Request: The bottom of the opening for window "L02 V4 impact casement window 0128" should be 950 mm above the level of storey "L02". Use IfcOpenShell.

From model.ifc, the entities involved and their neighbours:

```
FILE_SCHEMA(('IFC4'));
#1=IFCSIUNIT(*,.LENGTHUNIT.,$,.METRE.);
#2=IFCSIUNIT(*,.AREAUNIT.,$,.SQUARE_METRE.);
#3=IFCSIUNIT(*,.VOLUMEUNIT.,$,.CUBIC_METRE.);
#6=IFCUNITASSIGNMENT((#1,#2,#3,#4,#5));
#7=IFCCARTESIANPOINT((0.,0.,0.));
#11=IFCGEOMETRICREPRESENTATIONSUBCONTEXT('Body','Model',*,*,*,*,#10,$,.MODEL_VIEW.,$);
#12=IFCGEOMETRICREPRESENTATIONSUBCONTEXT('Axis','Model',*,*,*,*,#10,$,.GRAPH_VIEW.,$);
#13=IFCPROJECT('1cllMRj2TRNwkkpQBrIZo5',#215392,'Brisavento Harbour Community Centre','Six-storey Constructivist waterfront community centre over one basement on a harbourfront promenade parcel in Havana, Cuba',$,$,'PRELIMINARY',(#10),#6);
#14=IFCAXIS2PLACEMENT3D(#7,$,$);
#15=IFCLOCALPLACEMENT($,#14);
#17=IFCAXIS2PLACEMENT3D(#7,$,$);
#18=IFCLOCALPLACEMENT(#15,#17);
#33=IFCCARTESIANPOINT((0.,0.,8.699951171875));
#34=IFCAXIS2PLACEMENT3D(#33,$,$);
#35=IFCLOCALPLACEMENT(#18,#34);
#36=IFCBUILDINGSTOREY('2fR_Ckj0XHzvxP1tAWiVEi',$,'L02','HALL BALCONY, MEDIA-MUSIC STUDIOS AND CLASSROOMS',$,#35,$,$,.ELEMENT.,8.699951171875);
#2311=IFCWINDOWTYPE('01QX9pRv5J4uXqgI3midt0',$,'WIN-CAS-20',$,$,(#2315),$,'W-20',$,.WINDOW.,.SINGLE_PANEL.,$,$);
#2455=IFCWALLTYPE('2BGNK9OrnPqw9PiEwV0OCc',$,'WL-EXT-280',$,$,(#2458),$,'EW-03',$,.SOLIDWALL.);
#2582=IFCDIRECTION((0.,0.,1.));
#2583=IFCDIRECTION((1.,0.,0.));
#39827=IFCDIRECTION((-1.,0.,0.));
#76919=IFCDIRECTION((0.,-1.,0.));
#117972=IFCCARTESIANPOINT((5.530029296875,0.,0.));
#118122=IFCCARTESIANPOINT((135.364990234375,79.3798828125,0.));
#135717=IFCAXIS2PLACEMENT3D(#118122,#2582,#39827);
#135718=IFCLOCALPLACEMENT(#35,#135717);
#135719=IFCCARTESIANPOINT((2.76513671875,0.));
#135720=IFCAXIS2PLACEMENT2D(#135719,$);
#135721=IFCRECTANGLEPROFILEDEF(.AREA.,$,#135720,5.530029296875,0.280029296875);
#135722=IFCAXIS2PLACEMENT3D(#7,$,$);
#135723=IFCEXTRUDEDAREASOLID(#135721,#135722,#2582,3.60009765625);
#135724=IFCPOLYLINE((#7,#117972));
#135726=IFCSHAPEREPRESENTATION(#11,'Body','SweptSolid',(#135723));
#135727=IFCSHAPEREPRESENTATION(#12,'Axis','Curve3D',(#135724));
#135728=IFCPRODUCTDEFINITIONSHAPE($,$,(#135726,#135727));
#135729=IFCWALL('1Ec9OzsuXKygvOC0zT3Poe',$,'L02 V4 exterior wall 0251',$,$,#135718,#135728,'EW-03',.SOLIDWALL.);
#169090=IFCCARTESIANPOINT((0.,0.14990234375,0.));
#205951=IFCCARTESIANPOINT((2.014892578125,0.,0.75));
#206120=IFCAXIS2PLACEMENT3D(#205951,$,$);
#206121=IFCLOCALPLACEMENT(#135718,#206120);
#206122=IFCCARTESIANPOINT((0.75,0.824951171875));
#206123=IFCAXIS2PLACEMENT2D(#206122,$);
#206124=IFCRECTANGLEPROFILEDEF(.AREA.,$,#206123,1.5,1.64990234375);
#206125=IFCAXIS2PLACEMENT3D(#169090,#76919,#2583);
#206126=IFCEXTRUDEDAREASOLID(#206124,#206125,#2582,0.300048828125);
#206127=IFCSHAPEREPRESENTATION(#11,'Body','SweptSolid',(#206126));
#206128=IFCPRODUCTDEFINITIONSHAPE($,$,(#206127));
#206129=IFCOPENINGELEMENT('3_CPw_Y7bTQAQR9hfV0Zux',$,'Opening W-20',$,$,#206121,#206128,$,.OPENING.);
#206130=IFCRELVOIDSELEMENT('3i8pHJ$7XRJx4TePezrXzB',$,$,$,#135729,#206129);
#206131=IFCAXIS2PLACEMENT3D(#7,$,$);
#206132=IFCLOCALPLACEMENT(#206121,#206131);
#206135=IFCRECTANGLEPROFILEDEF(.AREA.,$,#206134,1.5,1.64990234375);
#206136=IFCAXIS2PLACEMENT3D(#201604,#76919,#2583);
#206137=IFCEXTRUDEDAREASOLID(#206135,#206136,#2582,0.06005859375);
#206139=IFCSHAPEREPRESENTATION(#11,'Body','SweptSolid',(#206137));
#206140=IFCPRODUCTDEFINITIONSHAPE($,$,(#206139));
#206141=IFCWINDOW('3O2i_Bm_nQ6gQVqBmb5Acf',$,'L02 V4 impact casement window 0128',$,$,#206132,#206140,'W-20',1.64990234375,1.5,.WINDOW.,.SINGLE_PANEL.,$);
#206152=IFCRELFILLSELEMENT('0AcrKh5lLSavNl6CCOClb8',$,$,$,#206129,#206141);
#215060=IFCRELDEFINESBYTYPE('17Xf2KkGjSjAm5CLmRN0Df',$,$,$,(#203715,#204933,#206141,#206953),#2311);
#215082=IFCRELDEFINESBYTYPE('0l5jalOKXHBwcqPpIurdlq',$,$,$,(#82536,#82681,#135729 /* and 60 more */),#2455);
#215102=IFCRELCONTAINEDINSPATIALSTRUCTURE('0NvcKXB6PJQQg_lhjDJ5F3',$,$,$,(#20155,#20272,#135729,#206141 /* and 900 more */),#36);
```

```python
import numpy as np
import ifcopenshell
import ifcopenshell.api.geometry
import ifcopenshell.geom
import ifcopenshell.util.element
import ifcopenshell.util.placement
import ifcopenshell.util.shape
import ifcopenshell.util.unit

model = ifcopenshell.open("model.ifc")
unit_scale = ifcopenshell.util.unit.calculate_unit_scale(model)

window = model.by_guid("3O2i_Bm_nQ6gQVqBmb5Acf")
opening = window.FillsVoids[0].RelatingOpeningElement
storey = ifcopenshell.util.element.get_container(window, ifc_class="IfcBuildingStorey")
level = ifcopenshell.util.placement.get_local_placement(storey.ObjectPlacement)[2, 3]

# The opening's origin need not be at the sill, so measure its lowest point.
shape = ifcopenshell.geom.create_shape(ifcopenshell.geom.settings(), opening)
bottom = ifcopenshell.util.shape.get_shape_bottom_elevation(shape, shape.geometry) / unit_scale
dz = level + 0.95 / unit_scale - bottom

shift = np.array([0.0, 0.0, dz])
# The window is placed relative to its opening, so it follows when the opening moves.
matrix = ifcopenshell.util.placement.get_local_placement(opening.ObjectPlacement)
matrix[:3, 3] += shift
ifcopenshell.api.geometry.edit_object_placement(
    model, product=opening, matrix=matrix, is_si=False, should_transform_children=True
)

print(f"moved by {dz * unit_scale:+.3f} m")

model.write("model_updated.ifc")
```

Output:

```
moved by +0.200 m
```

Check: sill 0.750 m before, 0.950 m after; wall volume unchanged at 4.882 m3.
